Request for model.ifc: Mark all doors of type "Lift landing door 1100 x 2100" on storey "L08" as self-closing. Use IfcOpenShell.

First a look at what the model holds.

```python
import ifcopenshell
import ifcopenshell.util.element

model = ifcopenshell.open("model.ifc")
print(model.schema)
storey = next(s for s in model.by_type("IfcBuildingStorey") if s.Name == "L08")
doors = [e for e in ifcopenshell.util.element.get_decomposition(storey) if e.is_a("IfcDoor")]
seen = {}
for e in doors:
    element_type = ifcopenshell.util.element.get_type(e)
    key = (element_type.Name if element_type != e and element_type else None, ifcopenshell.util.element.get_pset(e, "Pset_DoorCommon", "SelfClosing"))
    seen[key] = seen.get(key, 0) + 1
for (name, value), count in sorted(seen.items(), key=str):
    print(count, "x", name, "|", value)
```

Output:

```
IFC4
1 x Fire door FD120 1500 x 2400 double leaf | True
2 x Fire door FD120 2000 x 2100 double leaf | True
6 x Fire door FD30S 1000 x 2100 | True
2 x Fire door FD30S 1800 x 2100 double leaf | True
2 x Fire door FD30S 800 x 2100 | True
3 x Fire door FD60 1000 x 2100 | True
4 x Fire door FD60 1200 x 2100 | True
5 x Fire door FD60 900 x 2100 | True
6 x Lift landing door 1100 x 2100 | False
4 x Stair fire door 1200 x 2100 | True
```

```python
import ifcopenshell
import ifcopenshell.api.pset
import ifcopenshell.util.element

model = ifcopenshell.open("model.ifc")

storey = next(s for s in model.by_type("IfcBuildingStorey") if s.Name == "L08")
doors = [e for e in ifcopenshell.util.element.get_decomposition(storey) if e.is_a("IfcDoor")]

count = 0
for e in doors:
    element_type = ifcopenshell.util.element.get_type(e)
    if element_type in (None, e) or element_type.Name != "Lift landing door 1100 x 2100":
        continue
    # add_pset returns the element's existing set when there is one.
    pset = ifcopenshell.api.pset.add_pset(model, product=e, name="Pset_DoorCommon")
    ifcopenshell.api.pset.edit_pset(model, pset=pset, properties={"SelfClosing": True})
    count += 1

print(count, "doors updated")

model.write("model-out.ifc")
```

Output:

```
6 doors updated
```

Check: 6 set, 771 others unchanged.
